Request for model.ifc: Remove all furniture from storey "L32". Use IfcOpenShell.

First a look at what the model holds.

```python
import ifcopenshell
import ifcopenshell.util.element

model = ifcopenshell.open("model.ifc")
print(model.schema)
storey = next(s for s in model.by_type("IfcBuildingStorey") if s.Name == "L32")
furniture = [e for e in ifcopenshell.util.element.get_decomposition(storey) if e.is_a("IfcFurnishingElement")]
seen = {}
for e in furniture:
    element_type = ifcopenshell.util.element.get_type(e)
    name = element_type.Name if element_type not in (None, e) else None
    seen[name] = seen.get(name, 0) + 1
for name, count in sorted(seen.items(), key=str):
    print(count, "x", name)
```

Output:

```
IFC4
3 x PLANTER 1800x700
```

```python
import ifcopenshell
import ifcopenshell.api.root
import ifcopenshell.util.element

model = ifcopenshell.open("model.ifc")

storey = next(s for s in model.by_type("IfcBuildingStorey") if s.Name == "L32")
furniture = [e for e in ifcopenshell.util.element.get_decomposition(storey) if e.is_a("IfcFurnishingElement")]

for e in furniture:
    ifcopenshell.api.root.remove_product(model, product=e)
print(len(furniture), "removed")

model.write("model-out.ifc")
```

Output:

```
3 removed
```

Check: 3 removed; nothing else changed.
